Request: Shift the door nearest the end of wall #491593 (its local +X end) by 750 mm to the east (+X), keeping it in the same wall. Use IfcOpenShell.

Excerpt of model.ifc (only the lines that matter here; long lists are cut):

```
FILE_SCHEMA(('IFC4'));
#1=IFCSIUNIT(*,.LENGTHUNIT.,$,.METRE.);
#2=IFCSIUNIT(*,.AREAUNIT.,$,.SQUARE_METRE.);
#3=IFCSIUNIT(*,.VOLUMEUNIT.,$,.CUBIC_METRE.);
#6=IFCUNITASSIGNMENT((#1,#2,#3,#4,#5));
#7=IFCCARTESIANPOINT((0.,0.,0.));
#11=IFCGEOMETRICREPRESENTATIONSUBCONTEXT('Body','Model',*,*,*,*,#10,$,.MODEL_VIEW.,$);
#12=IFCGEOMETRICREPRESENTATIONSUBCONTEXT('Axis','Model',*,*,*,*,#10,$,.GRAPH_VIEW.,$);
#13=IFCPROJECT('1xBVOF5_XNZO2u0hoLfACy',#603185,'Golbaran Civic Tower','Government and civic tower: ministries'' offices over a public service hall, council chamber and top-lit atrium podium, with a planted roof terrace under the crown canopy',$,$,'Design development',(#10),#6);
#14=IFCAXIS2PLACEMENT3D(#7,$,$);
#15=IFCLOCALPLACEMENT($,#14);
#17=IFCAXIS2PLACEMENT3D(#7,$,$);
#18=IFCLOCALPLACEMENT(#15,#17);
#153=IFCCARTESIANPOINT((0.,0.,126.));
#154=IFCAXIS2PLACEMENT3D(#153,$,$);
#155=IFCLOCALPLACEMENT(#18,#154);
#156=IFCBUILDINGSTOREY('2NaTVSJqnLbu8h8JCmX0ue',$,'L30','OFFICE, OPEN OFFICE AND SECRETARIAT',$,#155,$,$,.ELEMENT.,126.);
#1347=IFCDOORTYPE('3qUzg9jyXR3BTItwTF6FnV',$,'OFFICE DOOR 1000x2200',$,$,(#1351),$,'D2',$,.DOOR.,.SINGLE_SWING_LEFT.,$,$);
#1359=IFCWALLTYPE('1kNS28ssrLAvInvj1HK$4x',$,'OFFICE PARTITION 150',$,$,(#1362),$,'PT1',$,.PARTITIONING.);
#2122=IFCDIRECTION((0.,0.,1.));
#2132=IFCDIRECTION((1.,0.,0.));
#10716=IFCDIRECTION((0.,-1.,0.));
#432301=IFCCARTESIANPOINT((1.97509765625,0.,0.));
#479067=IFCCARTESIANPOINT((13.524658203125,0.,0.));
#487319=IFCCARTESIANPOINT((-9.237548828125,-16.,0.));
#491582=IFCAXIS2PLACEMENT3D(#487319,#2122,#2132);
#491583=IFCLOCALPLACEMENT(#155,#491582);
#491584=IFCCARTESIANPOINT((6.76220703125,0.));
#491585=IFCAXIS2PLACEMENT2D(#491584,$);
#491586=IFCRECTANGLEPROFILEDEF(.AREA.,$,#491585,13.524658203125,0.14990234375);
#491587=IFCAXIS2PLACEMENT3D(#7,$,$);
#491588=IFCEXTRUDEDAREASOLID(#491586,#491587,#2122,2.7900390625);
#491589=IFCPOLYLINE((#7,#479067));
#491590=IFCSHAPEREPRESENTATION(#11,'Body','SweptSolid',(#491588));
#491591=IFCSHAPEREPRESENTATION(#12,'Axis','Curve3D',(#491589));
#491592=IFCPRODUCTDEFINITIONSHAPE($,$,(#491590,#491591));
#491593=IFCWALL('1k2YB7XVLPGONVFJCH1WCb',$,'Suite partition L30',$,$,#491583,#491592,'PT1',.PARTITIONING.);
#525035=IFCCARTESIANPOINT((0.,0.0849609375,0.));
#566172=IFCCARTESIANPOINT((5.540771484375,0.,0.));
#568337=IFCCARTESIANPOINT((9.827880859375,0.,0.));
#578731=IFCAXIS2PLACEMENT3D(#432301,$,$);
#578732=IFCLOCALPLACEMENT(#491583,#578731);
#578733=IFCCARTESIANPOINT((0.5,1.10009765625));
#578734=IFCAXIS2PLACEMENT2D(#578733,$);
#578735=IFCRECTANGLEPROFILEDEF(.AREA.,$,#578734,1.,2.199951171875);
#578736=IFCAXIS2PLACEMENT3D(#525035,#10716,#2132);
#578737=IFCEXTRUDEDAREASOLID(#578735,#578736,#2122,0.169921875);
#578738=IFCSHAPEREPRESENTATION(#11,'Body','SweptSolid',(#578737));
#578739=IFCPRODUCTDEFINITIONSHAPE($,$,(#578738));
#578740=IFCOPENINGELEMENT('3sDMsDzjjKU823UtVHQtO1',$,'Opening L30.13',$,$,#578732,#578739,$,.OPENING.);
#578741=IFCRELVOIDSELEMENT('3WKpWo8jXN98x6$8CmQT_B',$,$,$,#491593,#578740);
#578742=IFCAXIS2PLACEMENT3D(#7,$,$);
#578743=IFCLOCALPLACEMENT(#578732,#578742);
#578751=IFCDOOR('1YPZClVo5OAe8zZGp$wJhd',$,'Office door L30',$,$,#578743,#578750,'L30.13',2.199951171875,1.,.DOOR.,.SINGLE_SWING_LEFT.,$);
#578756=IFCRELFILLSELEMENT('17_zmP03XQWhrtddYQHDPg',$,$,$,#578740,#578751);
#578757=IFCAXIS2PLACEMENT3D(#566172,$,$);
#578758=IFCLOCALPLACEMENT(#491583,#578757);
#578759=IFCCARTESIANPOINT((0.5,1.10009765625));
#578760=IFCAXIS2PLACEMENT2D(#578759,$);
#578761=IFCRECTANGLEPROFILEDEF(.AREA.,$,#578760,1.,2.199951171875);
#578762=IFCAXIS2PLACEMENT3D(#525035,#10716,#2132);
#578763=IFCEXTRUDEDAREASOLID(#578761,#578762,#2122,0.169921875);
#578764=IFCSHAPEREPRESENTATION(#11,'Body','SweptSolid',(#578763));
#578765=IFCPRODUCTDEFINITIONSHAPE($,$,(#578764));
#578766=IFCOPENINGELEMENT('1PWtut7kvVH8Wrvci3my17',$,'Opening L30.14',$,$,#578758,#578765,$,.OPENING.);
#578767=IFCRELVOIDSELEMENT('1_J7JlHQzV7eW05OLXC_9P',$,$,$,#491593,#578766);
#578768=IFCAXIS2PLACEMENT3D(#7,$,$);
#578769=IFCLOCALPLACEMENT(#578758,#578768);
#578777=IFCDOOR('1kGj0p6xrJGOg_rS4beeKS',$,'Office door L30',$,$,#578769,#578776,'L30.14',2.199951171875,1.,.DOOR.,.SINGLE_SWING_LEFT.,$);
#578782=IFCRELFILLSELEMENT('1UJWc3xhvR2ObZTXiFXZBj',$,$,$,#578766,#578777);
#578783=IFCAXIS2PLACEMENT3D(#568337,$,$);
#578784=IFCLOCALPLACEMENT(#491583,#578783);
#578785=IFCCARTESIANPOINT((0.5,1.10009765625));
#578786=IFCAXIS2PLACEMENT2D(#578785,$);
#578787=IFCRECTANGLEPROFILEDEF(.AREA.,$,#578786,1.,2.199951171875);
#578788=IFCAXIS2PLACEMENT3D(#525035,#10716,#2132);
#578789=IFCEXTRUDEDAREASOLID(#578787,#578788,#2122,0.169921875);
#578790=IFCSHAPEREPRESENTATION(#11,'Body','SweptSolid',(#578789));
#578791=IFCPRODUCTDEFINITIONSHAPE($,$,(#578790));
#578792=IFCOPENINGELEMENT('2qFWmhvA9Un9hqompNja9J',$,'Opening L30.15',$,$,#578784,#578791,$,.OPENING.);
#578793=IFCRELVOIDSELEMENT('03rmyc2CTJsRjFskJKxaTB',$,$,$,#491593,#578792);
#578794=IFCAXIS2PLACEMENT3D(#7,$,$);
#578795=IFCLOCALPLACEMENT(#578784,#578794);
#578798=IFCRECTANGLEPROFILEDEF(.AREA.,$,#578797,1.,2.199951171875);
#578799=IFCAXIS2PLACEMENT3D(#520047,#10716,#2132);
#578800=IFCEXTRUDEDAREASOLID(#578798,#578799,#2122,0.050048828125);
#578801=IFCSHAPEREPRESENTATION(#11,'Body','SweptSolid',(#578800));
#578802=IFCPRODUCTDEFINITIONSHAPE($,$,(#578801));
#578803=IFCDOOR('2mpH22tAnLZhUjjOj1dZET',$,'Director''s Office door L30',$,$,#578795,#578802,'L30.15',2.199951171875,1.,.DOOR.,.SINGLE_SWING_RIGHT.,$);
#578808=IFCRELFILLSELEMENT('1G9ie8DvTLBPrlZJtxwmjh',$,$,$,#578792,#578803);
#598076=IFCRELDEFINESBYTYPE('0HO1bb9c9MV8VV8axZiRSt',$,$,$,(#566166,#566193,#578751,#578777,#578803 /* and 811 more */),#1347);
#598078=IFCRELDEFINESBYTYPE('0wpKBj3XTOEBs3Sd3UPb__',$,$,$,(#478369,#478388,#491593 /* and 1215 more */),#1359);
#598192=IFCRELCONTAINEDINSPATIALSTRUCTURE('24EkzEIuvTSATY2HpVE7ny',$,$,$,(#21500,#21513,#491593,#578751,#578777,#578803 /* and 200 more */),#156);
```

```python
import ifcopenshell
import ifcopenshell.api.geometry
import ifcopenshell.util.placement
import ifcopenshell.util.unit

model = ifcopenshell.open("model.ifc")
unit_scale = ifcopenshell.util.unit.calculate_unit_scale(model)

door = model.by_guid("2mpH22tAnLZhUjjOj1dZET")
opening = door.FillsVoids[0].RelatingOpeningElement
wall = opening.VoidsElements[0].RelatingBuildingElement

wall_matrix = ifcopenshell.util.placement.get_local_placement(wall.ObjectPlacement)
shift = wall_matrix[:3, 0] * 0.75 / unit_scale
before = ifcopenshell.util.placement.get_local_placement(door.ObjectPlacement)[:3, 3].copy()

# The door is placed relative to its opening, so it follows when the opening moves.
matrix = ifcopenshell.util.placement.get_local_placement(opening.ObjectPlacement)
matrix[:3, 3] += shift
ifcopenshell.api.geometry.edit_object_placement(
    model, product=opening, matrix=matrix, is_si=False, should_transform_children=True
)

after = ifcopenshell.util.placement.get_local_placement(door.ObjectPlacement)[:3, 3]
print("door moved by", (after - before).round(3) + 0.0)

model.write("model_rev.ifc")
```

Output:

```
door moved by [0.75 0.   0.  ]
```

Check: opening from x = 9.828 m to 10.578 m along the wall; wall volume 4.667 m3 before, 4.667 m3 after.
